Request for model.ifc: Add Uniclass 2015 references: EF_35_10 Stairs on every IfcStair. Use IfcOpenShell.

First a look at what the model holds.

```python
import ifcopenshell

model = ifcopenshell.open("model.ifc")
print(model.schema)
print("classifications:", [c.Name for c in model.by_type("IfcClassification")])
for ifc_class in ("IfcDoor", "IfcRoof", "IfcStair", "IfcWall", "IfcWindow"):
    print(ifc_class, len(model.by_type(ifc_class)))
```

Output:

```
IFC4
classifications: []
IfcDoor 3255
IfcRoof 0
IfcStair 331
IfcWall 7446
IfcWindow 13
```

```python
import ifcopenshell
import ifcopenshell.api.classification

model = ifcopenshell.open("model.ifc")

system = ifcopenshell.api.classification.add_classification(model, classification="Uniclass 2015")

codes = {
    "IfcStair": ("EF_35_10", "Stairs"),
}
for ifc_class, (code, name) in codes.items():
    products = model.by_type(ifc_class)
    ifcopenshell.api.classification.add_reference(
        model, products=products, classification=system, identification=code, name=name
    )
    print(code, len(products))

model.write("model_updated.ifc")
```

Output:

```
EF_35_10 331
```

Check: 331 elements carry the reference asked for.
